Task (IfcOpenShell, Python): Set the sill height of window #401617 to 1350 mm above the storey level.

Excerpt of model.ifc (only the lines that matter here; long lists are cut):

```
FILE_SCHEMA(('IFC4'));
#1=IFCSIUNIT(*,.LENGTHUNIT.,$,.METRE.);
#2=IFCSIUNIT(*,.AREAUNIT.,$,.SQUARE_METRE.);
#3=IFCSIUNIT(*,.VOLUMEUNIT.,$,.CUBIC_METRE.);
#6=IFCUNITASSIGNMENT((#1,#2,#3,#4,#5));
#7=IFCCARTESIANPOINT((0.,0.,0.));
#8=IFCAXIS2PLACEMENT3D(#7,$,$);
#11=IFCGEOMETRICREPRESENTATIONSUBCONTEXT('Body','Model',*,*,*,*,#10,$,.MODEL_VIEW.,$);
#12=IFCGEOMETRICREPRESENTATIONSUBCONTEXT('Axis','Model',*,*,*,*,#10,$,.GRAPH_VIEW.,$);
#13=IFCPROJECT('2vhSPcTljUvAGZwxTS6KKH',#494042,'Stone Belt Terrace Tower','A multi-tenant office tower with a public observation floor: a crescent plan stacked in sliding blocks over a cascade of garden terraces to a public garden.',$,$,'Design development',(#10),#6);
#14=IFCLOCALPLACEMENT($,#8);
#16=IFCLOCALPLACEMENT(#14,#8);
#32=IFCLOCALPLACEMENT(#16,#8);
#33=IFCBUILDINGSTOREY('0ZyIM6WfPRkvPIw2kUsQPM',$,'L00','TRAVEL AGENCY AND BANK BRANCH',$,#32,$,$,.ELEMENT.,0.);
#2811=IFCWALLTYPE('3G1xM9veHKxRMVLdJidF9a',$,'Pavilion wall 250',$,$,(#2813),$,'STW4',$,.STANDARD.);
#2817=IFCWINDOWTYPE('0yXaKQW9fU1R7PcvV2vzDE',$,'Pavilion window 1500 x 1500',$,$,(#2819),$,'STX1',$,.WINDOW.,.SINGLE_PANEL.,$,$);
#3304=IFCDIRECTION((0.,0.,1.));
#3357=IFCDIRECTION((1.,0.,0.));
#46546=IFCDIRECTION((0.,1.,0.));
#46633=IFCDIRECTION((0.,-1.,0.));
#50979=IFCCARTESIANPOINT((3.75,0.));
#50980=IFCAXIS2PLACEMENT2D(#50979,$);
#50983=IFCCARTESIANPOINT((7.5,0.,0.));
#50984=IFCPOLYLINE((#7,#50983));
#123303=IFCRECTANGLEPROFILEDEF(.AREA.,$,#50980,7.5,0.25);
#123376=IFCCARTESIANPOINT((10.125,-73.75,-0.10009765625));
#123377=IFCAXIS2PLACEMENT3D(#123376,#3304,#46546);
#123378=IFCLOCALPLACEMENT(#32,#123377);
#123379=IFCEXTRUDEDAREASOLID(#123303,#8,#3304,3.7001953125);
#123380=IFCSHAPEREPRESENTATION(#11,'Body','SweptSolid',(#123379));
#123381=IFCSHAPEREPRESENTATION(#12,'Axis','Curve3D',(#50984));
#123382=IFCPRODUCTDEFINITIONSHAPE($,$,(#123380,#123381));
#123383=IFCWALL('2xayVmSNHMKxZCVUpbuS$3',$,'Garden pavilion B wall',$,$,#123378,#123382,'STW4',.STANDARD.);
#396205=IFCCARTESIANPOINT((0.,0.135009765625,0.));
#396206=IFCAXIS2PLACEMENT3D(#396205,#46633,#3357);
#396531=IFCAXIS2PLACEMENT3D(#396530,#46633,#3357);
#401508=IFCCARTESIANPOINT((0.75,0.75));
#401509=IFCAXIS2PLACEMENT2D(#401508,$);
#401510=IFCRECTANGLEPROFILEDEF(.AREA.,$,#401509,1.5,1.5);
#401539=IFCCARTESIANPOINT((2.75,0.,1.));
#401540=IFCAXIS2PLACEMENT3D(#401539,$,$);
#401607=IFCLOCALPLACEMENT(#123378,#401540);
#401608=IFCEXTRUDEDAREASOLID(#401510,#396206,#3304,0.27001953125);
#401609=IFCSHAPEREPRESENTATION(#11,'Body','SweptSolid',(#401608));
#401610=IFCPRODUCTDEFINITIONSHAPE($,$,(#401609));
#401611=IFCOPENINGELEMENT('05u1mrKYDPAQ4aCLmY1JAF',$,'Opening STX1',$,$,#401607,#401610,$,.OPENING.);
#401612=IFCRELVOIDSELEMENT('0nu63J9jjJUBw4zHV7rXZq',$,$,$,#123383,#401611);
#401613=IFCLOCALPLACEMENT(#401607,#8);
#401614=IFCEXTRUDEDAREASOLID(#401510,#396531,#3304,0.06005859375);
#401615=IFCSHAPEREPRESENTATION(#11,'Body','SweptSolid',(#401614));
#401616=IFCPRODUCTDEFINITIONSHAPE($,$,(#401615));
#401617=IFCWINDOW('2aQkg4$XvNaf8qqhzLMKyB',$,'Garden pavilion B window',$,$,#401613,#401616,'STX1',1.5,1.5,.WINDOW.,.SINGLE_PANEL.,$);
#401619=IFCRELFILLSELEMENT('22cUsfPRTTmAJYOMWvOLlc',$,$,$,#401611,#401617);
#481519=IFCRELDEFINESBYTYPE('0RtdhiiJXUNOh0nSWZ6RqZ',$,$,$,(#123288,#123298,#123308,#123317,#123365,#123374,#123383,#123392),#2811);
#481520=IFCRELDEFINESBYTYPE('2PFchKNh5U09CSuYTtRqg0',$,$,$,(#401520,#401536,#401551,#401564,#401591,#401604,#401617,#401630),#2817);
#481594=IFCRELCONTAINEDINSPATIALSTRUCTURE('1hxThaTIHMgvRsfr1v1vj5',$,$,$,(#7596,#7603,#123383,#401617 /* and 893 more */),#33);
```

```python
import numpy as np
import ifcopenshell
import ifcopenshell.api.geometry
import ifcopenshell.geom
import ifcopenshell.util.element
import ifcopenshell.util.placement
import ifcopenshell.util.shape
import ifcopenshell.util.unit

model = ifcopenshell.open("model.ifc")
unit_scale = ifcopenshell.util.unit.calculate_unit_scale(model)

window = model.by_id(401617)
opening = window.FillsVoids[0].RelatingOpeningElement
storey = ifcopenshell.util.element.get_container(window, ifc_class="IfcBuildingStorey")
level = ifcopenshell.util.placement.get_local_placement(storey.ObjectPlacement)[2, 3]

# The opening's origin need not be at the sill, so measure its lowest point.
shape = ifcopenshell.geom.create_shape(ifcopenshell.geom.settings(), opening)
bottom = ifcopenshell.util.shape.get_shape_bottom_elevation(shape, shape.geometry) / unit_scale
dz = level + 1.35 / unit_scale - bottom

shift = np.array([0.0, 0.0, dz])
# The window is placed relative to its opening, so it follows when the opening moves.
matrix = ifcopenshell.util.placement.get_local_placement(opening.ObjectPlacement)
matrix[:3, 3] += shift
ifcopenshell.api.geometry.edit_object_placement(
    model, product=opening, matrix=matrix, is_si=False, should_transform_children=True
)

print(f"moved by {dz * unit_scale:+.3f} m")

model.write("model_edited.ifc")
```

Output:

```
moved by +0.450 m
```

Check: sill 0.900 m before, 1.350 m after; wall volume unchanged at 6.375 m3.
